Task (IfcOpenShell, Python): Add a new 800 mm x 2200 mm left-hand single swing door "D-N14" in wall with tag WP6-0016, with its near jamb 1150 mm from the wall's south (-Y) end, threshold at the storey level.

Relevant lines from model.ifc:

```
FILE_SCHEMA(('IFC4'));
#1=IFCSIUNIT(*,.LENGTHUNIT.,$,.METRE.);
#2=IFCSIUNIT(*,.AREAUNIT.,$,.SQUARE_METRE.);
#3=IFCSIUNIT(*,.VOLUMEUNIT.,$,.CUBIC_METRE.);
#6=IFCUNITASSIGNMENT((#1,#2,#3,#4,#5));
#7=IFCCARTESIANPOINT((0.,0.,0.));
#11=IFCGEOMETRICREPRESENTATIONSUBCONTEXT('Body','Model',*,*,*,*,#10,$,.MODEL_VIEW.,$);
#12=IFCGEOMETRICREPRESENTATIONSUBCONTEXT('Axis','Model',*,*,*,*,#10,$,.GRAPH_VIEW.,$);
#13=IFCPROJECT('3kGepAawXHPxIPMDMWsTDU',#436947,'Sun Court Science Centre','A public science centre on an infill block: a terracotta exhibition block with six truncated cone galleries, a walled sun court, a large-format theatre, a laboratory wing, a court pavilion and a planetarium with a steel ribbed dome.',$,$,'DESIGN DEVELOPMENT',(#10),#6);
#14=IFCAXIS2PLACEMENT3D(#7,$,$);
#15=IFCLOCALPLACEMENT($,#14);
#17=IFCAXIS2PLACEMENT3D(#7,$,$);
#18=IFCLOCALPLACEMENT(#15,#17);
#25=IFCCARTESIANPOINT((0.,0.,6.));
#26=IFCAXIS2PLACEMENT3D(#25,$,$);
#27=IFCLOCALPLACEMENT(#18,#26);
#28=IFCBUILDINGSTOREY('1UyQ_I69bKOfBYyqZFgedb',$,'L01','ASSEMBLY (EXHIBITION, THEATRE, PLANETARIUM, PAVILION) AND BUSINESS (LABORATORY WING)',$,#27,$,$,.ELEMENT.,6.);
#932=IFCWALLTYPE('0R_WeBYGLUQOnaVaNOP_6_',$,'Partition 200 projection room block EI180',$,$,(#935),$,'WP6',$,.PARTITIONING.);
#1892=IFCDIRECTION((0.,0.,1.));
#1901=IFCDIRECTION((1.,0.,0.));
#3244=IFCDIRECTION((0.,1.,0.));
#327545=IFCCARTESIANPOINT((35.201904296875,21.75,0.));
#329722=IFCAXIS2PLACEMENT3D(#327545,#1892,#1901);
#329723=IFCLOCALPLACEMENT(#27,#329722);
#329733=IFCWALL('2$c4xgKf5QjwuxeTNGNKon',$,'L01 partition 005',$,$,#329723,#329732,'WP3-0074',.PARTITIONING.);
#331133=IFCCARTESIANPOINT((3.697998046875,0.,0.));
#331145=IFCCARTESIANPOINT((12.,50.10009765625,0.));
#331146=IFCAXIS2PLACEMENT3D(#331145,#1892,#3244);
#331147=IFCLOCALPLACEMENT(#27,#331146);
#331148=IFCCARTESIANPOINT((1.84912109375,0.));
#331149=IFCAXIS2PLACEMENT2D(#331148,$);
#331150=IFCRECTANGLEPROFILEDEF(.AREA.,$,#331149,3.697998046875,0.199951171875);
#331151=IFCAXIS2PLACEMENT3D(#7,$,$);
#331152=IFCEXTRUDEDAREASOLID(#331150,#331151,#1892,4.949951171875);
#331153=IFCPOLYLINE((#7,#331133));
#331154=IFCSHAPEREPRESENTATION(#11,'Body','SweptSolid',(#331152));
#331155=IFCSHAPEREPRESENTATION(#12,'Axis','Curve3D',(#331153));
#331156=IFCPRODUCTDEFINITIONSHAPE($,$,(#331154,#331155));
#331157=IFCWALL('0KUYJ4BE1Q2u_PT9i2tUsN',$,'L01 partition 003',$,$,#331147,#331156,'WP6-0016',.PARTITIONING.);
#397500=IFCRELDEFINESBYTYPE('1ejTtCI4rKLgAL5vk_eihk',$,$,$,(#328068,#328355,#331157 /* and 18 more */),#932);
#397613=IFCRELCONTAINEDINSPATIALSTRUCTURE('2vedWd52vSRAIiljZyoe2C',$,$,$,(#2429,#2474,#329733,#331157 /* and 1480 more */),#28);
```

```python
import numpy as np
import ifcopenshell
import ifcopenshell.api.feature
import ifcopenshell.api.geometry
import ifcopenshell.api.root
import ifcopenshell.api.spatial
import ifcopenshell.geom
import ifcopenshell.util.element
import ifcopenshell.util.placement
import ifcopenshell.util.representation
import ifcopenshell.util.shape
import ifcopenshell.util.unit

model = ifcopenshell.open("model.ifc")
unit_scale = ifcopenshell.util.unit.calculate_unit_scale(model)
settings = ifcopenshell.geom.settings()


def volume(element):
    """Net volume in cubic metres, openings subtracted."""
    shape = ifcopenshell.geom.create_shape(settings, element)
    return ifcopenshell.util.shape.get_volume(shape.geometry)


wall = model.by_id(331157)
storey = ifcopenshell.util.element.get_container(wall, ifc_class="IfcBuildingStorey")
context = ifcopenshell.util.representation.get_context(model, "Model", "Body", "MODEL_VIEW")
before = volume(wall)

width, height, from_end, sill = 0.8, 2.2, 1.15, 0.0  # metres

# The wall runs along its own X axis, and the end named is its -X end.
wall_shape = ifcopenshell.geom.create_shape(settings, wall)
x, y, z = ifcopenshell.util.shape.get_vertices(wall_shape.geometry).T
start = x.min() + from_end
face, thickness = float(y.min()), float(y.max() - y.min())
wall_matrix = ifcopenshell.util.placement.get_local_placement(wall.ObjectPlacement)
level = ifcopenshell.util.placement.get_local_placement(storey.ObjectPlacement)[2, 3]


def in_wall(x, y):
    """Placement at x, y metres in the wall's axes, at sill height."""
    matrix = wall_matrix.copy()
    matrix[:, 3] = wall_matrix @ np.array([x / unit_scale, y / unit_scale, 0.0, 1.0])
    matrix[2, 3] = level + sill / unit_scale
    return matrix


# Opening: a box that overshoots both wall faces by 50 mm.
opening = ifcopenshell.api.root.create_entity(model, ifc_class="IfcOpeningElement", predefined_type="OPENING")
box = ifcopenshell.api.geometry.add_wall_representation(
    model, context=context, length=width, height=height, thickness=thickness + 0.1
)
ifcopenshell.api.geometry.assign_representation(model, product=opening, representation=box)
ifcopenshell.api.geometry.edit_object_placement(model, product=opening, matrix=in_wall(start, face - 0.05), is_si=False)
ifcopenshell.api.feature.add_feature(model, feature=opening, element=wall)

door = ifcopenshell.api.root.create_entity(model, ifc_class="IfcDoor", name="D-N14", predefined_type="DOOR")
door.OverallWidth, door.OverallHeight = width / unit_scale, height / unit_scale
door.OperationType = "SINGLE_SWING_LEFT"
body = ifcopenshell.api.geometry.add_door_representation(
    model,
    context=context,
    overall_width=door.OverallWidth,
    overall_height=door.OverallHeight,
    operation_type="SINGLE_SWING_LEFT",
    lining_properties={"LiningDepth": thickness / unit_scale, "ThresholdDepth": thickness / unit_scale},
)
ifcopenshell.api.geometry.assign_representation(model, product=door, representation=body)
ifcopenshell.api.spatial.assign_container(model, products=[door], relating_structure=storey)
ifcopenshell.api.feature.add_filling(model, opening=opening, element=door)

# The lining spans the wall, so the door starts at the wall face.
ifcopenshell.api.geometry.edit_object_placement(model, product=door, matrix=in_wall(start, face), is_si=False)

after = volume(wall)

print(f"wall volume {before:.3f} -> {after:.3f} m3")

model.write("model-out.ifc")
```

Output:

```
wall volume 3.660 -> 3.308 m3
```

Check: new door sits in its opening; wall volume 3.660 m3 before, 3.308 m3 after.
